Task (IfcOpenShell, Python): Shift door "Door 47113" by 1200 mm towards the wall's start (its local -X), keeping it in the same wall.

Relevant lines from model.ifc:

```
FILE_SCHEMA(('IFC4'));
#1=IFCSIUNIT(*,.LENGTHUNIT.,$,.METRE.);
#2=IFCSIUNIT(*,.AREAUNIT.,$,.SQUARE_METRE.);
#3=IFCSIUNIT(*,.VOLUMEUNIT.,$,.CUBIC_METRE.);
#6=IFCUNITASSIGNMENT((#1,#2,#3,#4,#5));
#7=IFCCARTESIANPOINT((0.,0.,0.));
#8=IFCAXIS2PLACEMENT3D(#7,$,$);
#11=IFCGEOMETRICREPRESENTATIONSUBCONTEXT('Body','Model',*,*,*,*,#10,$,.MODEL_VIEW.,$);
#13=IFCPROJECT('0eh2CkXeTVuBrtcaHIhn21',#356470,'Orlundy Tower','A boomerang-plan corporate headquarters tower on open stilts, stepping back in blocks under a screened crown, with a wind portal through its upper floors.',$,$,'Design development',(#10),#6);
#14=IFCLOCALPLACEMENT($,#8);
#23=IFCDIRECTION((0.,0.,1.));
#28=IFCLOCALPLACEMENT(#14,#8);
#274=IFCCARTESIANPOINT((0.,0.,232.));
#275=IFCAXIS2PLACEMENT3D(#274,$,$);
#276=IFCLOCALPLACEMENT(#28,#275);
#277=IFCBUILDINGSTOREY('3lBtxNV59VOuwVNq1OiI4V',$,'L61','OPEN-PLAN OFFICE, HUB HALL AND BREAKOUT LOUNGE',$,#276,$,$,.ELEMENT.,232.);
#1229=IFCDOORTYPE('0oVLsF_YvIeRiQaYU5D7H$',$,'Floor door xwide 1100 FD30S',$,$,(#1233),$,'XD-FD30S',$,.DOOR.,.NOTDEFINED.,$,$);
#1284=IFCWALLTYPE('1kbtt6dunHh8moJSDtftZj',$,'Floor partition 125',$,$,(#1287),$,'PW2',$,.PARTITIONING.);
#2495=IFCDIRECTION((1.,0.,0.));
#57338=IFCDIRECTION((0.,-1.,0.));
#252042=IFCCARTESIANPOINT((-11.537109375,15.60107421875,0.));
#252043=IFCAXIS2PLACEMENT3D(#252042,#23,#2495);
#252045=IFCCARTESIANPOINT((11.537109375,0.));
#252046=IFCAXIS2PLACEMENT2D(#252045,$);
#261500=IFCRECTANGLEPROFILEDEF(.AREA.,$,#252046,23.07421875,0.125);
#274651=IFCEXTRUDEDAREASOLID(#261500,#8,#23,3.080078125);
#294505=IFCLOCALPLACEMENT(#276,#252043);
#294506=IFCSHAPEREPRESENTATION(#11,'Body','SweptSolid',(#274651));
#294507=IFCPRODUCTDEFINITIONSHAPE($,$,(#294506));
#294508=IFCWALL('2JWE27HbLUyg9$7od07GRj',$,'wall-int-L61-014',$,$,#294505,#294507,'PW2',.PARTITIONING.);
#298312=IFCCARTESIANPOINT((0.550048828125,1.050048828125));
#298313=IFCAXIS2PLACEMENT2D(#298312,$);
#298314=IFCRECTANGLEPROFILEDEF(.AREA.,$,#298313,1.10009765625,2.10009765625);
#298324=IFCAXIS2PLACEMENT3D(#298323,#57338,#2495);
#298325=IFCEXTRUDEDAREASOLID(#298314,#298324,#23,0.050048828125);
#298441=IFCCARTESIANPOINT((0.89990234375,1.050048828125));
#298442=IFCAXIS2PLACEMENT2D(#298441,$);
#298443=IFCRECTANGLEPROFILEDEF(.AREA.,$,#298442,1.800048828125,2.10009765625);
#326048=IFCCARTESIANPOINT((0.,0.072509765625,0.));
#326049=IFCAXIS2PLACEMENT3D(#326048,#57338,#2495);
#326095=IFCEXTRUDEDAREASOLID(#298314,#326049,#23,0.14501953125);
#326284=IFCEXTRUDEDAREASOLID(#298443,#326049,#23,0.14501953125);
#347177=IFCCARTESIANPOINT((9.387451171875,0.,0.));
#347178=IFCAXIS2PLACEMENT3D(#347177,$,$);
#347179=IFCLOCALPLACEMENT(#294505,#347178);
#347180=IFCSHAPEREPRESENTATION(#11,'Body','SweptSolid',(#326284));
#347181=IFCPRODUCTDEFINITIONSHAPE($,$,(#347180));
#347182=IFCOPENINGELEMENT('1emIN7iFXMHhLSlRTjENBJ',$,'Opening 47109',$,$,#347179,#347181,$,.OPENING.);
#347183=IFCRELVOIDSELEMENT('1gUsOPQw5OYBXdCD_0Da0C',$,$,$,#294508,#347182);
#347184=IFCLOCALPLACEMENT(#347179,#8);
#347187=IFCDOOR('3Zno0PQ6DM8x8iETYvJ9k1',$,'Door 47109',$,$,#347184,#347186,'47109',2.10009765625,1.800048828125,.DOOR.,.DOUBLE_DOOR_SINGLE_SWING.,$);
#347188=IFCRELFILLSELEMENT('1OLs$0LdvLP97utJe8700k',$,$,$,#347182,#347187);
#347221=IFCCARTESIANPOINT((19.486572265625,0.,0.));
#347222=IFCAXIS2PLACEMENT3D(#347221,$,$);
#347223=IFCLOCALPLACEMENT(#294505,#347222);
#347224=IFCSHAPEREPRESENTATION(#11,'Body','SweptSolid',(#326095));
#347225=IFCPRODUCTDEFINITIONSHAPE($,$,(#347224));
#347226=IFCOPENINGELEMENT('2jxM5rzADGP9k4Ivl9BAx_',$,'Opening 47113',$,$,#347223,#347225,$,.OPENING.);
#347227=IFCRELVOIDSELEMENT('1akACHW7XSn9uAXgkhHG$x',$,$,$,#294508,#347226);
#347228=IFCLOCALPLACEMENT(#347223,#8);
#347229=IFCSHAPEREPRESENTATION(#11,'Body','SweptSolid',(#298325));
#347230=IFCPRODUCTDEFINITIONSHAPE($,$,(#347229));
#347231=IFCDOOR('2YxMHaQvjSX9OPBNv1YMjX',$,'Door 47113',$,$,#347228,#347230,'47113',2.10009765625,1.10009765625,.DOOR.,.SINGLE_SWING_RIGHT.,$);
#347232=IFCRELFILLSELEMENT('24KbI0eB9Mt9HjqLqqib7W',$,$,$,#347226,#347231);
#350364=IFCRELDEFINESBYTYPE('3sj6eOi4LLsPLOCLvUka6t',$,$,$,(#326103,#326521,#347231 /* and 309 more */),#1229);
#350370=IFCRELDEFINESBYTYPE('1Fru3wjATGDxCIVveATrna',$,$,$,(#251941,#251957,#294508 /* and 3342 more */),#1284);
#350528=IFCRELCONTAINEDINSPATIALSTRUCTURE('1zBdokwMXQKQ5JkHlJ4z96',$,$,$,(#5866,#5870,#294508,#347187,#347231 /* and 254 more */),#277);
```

```python
import ifcopenshell
import ifcopenshell.api.geometry
import ifcopenshell.util.placement
import ifcopenshell.util.unit

model = ifcopenshell.open("model.ifc")
unit_scale = ifcopenshell.util.unit.calculate_unit_scale(model)

door = model.by_id(347231)
opening = door.FillsVoids[0].RelatingOpeningElement
wall = opening.VoidsElements[0].RelatingBuildingElement

wall_matrix = ifcopenshell.util.placement.get_local_placement(wall.ObjectPlacement)
shift = wall_matrix[:3, 0] * -1.2 / unit_scale
before = ifcopenshell.util.placement.get_local_placement(door.ObjectPlacement)[:3, 3].copy()

# The door is placed relative to its opening, so it follows when the opening moves.
matrix = ifcopenshell.util.placement.get_local_placement(opening.ObjectPlacement)
matrix[:3, 3] += shift
ifcopenshell.api.geometry.edit_object_placement(
    model, product=opening, matrix=matrix, is_si=False, should_transform_children=True
)

after = ifcopenshell.util.placement.get_local_placement(door.ObjectPlacement)[:3, 3]
print("door moved by", (after - before).round(3) + 0.0)

model.write("model_rev.ifc")
```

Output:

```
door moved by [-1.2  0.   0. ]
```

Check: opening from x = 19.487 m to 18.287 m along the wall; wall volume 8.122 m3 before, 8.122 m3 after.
